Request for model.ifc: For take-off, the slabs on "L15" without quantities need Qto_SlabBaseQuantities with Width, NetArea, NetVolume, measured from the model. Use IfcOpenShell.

First a look at what the model holds.

```python
import ifcopenshell
import ifcopenshell.util.element
import ifcopenshell.util.unit

model = ifcopenshell.open("model.ifc")
print(model.schema)
for unit_type in ("LENGTHUNIT", "AREAUNIT", "VOLUMEUNIT"):
    print(unit_type, ifcopenshell.util.unit.calculate_unit_scale(model, unit_type))
storey = next(s for s in model.by_type("IfcBuildingStorey") if s.Name == "L15")
slabs = [e for e in ifcopenshell.util.element.get_decomposition(storey) if e.is_a("IfcSlab")]
for e in sorted(slabs, key=lambda e: e.id()):
    print(e.id(), e.is_a(), e.Name, list(ifcopenshell.util.element.get_psets(e, qtos_only=True)), sep=" | ")
```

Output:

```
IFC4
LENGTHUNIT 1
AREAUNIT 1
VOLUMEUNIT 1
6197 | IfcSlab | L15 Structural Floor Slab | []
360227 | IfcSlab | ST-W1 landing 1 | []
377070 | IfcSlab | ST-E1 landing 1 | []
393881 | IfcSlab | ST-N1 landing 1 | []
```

```python
import ifcopenshell
import ifcopenshell.api.pset
import ifcopenshell.geom
import ifcopenshell.util.element
import ifcopenshell.util.shape
import ifcopenshell.util.unit

model = ifcopenshell.open("model.ifc")
unit_scale = ifcopenshell.util.unit.calculate_unit_scale(model)
area_scale = ifcopenshell.util.unit.calculate_unit_scale(model, "AREAUNIT")
volume_scale = ifcopenshell.util.unit.calculate_unit_scale(model, "VOLUMEUNIT")
settings = ifcopenshell.geom.settings()

storey = next(s for s in model.by_type("IfcBuildingStorey") if s.Name == "L15")
slabs = [e for e in ifcopenshell.util.element.get_decomposition(storey) if e.is_a("IfcSlab")]

for e in sorted(slabs, key=lambda e: e.id()):
    if ifcopenshell.util.element.get_psets(e, qtos_only=True, should_inherit=False):
        continue
    # Geometry comes back in metres, in the element's own axes.
    shape = ifcopenshell.geom.create_shape(settings, e)
    values = {
        "Width": ifcopenshell.util.shape.get_z(shape.geometry) / unit_scale,
        "NetArea": ifcopenshell.util.shape.get_footprint_area(shape.geometry) / area_scale,
        "NetVolume": ifcopenshell.util.shape.get_volume(shape.geometry) / volume_scale,
    }
    qto = ifcopenshell.api.pset.add_qto(model, product=e, name="Qto_SlabBaseQuantities")
    ifcopenshell.api.pset.edit_qto(model, qto=qto, properties=values)
    print(e.id(), {k: round(v, 3) for k, v in values.items()})

model.write("model_rev.ifc")
```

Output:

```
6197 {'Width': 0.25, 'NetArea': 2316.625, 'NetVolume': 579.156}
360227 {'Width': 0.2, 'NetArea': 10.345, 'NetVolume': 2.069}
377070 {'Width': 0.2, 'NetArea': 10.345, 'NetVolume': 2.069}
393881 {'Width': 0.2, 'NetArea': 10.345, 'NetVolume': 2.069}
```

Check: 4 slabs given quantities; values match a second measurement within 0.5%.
